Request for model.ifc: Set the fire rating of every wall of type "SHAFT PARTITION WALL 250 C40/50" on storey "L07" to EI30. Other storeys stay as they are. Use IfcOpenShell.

First a look at what the model holds.

```python
import ifcopenshell
import ifcopenshell.util.element

model = ifcopenshell.open("model.ifc")
print(model.schema)
storey = next(s for s in model.by_type("IfcBuildingStorey") if s.Name == "L07")
walls = [e for e in ifcopenshell.util.element.get_decomposition(storey) if e.is_a("IfcWall")]
seen = {}
for e in walls:
    element_type = ifcopenshell.util.element.get_type(e)
    key = (element_type.Name if element_type != e and element_type else None, ifcopenshell.util.element.get_pset(e, "Pset_WallCommon", "FireRating"))
    seen[key] = seen.get(key, 0) + 1
for (name, value), count in sorted(seen.items(), key=str):
    print(count, "x", name, "|", value)
```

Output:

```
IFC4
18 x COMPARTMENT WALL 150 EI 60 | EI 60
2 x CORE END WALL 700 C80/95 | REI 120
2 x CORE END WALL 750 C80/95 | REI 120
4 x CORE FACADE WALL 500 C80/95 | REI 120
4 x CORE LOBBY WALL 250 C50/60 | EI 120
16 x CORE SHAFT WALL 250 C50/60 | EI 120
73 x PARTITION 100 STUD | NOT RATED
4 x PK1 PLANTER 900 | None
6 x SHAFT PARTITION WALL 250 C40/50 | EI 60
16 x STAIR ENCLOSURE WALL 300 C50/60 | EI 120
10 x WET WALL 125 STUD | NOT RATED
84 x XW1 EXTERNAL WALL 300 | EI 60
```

```python
import ifcopenshell
import ifcopenshell.api.pset
import ifcopenshell.util.element

model = ifcopenshell.open("model.ifc")

storey = next(s for s in model.by_type("IfcBuildingStorey") if s.Name == "L07")
walls = [e for e in ifcopenshell.util.element.get_decomposition(storey) if e.is_a("IfcWall")]

count = 0
for e in walls:
    element_type = ifcopenshell.util.element.get_type(e)
    if element_type in (None, e) or element_type.Name != "SHAFT PARTITION WALL 250 C40/50":
        continue
    found = ifcopenshell.util.element.get_pset(e, "Pset_WallCommon", should_inherit=False)
    if found:
        pset = model.by_id(found["id"])
        if len(ifcopenshell.util.element.get_elements_by_pset(pset)) > 1:
            pset = ifcopenshell.api.pset.unshare_pset(model, products=[e], pset=pset)[0]
    else:
        pset = ifcopenshell.api.pset.add_pset(model, product=e, name="Pset_WallCommon")
    ifcopenshell.api.pset.edit_pset(model, pset=pset, properties={"FireRating": "EI30"})
    count += 1

print(count, "walls updated")

model.write("model-out.ifc")
```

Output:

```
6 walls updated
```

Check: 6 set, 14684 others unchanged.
